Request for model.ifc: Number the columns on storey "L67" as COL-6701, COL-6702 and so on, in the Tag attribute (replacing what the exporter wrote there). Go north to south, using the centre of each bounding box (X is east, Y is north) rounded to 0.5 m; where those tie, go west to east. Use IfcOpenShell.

First a look at what the model holds.

```python
import ifcopenshell
import ifcopenshell.util.element
import ifcopenshell.util.placement

model = ifcopenshell.open("model.ifc")
print(model.schema)
storey = next(s for s in model.by_type("IfcBuildingStorey") if s.Name == "L67")
columns = [e for e in ifcopenshell.util.element.get_decomposition(storey) if e.is_a("IfcColumn")]
for e in sorted(columns, key=lambda e: e.id()):
    origin = ifcopenshell.util.placement.get_local_placement(e.ObjectPlacement)[:3, 3]
    print(e.id(), e.Tag, e.Name, origin.round(2) + 0.0, sep=" | ")
```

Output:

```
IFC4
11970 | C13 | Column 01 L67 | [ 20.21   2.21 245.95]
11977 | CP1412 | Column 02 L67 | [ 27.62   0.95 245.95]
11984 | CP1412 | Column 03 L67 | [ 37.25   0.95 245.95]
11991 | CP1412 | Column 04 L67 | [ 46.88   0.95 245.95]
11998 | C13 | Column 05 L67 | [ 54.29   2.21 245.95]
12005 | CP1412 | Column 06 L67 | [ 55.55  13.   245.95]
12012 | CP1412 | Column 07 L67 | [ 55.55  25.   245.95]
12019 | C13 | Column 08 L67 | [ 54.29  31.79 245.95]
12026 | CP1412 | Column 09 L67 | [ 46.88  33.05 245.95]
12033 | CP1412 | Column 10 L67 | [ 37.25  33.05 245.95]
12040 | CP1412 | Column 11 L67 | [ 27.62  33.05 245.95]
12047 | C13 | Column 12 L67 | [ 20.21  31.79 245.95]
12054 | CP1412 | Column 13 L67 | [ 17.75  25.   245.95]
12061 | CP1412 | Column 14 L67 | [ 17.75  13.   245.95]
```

```python
import ifcopenshell
import ifcopenshell.geom
import ifcopenshell.util.element
import ifcopenshell.util.shape

model = ifcopenshell.open("model.ifc")
settings = ifcopenshell.geom.settings()
settings.set("use-world-coords", True)


def centre(element):
    shape = ifcopenshell.geom.create_shape(settings, element)
    return ifcopenshell.util.shape.get_bbox_centroid(shape.geometry)


storey = next(s for s in model.by_type("IfcBuildingStorey") if s.Name == "L67")
columns = [e for e in ifcopenshell.util.element.get_decomposition(storey) if e.is_a("IfcColumn")]

# Insertion points can sit at a corner or the storey origin, so sort by the geometry (in metres).
centres = {e: centre(e) for e in columns}
columns.sort(key=lambda e: (-round(centres[e][1] / 0.5), centres[e][0]))

for i, e in enumerate(columns, start=1):
    number = f"COL-67{i:02d}"
    e.Tag = number
    print(e.id(), number)

model.write("model-out.ifc")
```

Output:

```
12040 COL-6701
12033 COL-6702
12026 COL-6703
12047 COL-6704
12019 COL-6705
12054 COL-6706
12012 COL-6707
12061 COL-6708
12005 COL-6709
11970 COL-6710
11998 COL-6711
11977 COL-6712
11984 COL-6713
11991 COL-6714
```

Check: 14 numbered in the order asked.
